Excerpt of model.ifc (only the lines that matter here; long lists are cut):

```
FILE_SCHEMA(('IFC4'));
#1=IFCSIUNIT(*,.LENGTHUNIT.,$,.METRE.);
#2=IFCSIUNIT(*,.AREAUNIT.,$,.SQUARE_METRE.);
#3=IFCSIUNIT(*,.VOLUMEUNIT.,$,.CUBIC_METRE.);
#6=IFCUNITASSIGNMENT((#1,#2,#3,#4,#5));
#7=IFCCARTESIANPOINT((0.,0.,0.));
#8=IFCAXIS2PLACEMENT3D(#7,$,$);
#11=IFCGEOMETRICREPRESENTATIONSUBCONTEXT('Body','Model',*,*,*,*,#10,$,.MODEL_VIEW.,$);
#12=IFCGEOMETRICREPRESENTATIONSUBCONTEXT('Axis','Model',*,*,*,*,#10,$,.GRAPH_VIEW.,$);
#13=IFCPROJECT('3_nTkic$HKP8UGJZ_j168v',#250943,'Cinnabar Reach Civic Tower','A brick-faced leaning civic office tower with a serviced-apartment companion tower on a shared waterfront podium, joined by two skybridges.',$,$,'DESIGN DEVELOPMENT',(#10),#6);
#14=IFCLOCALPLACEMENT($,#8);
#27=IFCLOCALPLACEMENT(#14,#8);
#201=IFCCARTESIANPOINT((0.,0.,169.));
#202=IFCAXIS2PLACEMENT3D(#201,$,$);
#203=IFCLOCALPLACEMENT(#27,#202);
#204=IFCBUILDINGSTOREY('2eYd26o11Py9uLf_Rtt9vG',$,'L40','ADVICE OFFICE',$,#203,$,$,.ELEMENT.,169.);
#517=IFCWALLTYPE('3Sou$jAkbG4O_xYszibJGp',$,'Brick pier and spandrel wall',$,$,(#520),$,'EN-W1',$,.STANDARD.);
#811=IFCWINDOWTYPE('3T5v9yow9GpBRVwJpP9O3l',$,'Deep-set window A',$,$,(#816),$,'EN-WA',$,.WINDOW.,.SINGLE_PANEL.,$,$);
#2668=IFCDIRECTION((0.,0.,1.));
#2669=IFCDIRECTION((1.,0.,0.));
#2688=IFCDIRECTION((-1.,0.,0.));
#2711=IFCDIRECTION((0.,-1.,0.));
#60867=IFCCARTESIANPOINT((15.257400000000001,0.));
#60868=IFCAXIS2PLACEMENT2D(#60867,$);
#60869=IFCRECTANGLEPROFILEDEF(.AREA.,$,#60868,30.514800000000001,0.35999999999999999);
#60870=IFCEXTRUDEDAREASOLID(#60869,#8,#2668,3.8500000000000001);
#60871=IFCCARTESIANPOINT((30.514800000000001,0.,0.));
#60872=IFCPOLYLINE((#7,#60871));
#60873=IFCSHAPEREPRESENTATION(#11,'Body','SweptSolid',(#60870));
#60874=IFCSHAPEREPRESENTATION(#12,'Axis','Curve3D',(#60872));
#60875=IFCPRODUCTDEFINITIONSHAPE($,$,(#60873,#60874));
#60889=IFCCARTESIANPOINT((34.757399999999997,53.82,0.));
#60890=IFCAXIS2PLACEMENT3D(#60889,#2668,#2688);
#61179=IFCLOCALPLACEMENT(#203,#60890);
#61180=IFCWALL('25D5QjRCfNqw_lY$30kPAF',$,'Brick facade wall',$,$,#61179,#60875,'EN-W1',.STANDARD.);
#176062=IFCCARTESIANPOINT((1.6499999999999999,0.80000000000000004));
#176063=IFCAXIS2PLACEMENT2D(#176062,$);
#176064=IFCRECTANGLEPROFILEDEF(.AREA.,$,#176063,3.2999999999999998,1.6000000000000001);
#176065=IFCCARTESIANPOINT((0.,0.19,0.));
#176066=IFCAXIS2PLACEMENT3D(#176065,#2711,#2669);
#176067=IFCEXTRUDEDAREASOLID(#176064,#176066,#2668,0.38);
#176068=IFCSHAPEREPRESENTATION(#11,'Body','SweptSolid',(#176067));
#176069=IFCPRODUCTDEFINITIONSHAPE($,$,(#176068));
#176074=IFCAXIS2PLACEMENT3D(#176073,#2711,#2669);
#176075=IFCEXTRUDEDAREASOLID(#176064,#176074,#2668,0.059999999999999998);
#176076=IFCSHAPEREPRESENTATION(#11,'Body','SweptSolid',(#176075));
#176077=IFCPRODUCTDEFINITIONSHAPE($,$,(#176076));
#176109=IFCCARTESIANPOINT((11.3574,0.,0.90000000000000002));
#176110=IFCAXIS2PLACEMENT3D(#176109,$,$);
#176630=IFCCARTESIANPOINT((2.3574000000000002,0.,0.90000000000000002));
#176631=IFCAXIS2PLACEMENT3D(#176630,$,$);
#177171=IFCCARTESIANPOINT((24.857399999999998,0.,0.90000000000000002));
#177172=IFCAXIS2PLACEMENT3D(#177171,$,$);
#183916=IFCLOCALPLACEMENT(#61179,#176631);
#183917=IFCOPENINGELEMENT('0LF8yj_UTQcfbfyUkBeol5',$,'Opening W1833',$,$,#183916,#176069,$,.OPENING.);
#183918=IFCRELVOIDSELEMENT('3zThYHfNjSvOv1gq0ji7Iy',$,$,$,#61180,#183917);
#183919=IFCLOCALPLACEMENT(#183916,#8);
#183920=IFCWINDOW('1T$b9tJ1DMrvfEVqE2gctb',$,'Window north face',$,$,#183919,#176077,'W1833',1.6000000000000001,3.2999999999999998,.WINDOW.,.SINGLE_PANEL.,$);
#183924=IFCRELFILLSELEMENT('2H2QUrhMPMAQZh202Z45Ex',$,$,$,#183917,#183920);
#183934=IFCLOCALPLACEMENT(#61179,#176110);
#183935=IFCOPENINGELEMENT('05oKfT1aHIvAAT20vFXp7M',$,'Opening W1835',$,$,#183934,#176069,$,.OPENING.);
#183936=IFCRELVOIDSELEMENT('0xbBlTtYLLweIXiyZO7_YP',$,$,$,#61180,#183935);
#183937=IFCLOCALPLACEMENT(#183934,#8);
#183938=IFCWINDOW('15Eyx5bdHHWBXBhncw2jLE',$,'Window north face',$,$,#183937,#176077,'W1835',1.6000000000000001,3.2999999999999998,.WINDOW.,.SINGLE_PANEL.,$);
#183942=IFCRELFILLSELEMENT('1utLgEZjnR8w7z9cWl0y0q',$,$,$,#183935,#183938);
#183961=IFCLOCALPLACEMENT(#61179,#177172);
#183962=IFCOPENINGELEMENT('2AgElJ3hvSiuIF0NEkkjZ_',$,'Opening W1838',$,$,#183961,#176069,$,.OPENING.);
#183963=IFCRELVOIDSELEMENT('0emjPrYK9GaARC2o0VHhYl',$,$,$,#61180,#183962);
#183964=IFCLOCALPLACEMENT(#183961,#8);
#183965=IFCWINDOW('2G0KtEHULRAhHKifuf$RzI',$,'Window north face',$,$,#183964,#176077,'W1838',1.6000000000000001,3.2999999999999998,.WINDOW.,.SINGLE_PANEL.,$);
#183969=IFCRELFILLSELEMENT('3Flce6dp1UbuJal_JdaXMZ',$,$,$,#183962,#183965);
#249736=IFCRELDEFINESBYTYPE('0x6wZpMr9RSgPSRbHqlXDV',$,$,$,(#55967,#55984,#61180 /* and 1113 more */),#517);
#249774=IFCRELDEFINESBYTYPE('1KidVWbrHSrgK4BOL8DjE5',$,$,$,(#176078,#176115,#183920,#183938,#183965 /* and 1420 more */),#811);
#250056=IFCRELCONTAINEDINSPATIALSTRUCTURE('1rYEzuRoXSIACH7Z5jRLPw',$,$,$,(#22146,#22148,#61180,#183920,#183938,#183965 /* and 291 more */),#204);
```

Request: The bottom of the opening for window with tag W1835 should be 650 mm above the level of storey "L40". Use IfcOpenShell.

```python
import numpy as np
import ifcopenshell
import ifcopenshell.api.geometry
import ifcopenshell.geom
import ifcopenshell.util.element
import ifcopenshell.util.placement
import ifcopenshell.util.shape
import ifcopenshell.util.unit

model = ifcopenshell.open("model.ifc")
unit_scale = ifcopenshell.util.unit.calculate_unit_scale(model)

window = model.by_guid("15Eyx5bdHHWBXBhncw2jLE")
opening = window.FillsVoids[0].RelatingOpeningElement
storey = ifcopenshell.util.element.get_container(window, ifc_class="IfcBuildingStorey")
level = ifcopenshell.util.placement.get_local_placement(storey.ObjectPlacement)[2, 3]

# The opening's origin need not be at the sill, so measure its lowest point.
shape = ifcopenshell.geom.create_shape(ifcopenshell.geom.settings(), opening)
bottom = ifcopenshell.util.shape.get_shape_bottom_elevation(shape, shape.geometry) / unit_scale
dz = level + 0.65 / unit_scale - bottom

shift = np.array([0.0, 0.0, dz])
# The window is placed relative to its opening, so it follows when the opening moves.
matrix = ifcopenshell.util.placement.get_local_placement(opening.ObjectPlacement)
matrix[:3, 3] += shift
ifcopenshell.api.geometry.edit_object_placement(
    model, product=opening, matrix=matrix, is_si=False, should_transform_children=True
)

print(f"moved by {dz * unit_scale:+.3f} m")

model.write("model_rev.ifc")
```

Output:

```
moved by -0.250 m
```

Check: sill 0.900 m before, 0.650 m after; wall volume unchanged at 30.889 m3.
